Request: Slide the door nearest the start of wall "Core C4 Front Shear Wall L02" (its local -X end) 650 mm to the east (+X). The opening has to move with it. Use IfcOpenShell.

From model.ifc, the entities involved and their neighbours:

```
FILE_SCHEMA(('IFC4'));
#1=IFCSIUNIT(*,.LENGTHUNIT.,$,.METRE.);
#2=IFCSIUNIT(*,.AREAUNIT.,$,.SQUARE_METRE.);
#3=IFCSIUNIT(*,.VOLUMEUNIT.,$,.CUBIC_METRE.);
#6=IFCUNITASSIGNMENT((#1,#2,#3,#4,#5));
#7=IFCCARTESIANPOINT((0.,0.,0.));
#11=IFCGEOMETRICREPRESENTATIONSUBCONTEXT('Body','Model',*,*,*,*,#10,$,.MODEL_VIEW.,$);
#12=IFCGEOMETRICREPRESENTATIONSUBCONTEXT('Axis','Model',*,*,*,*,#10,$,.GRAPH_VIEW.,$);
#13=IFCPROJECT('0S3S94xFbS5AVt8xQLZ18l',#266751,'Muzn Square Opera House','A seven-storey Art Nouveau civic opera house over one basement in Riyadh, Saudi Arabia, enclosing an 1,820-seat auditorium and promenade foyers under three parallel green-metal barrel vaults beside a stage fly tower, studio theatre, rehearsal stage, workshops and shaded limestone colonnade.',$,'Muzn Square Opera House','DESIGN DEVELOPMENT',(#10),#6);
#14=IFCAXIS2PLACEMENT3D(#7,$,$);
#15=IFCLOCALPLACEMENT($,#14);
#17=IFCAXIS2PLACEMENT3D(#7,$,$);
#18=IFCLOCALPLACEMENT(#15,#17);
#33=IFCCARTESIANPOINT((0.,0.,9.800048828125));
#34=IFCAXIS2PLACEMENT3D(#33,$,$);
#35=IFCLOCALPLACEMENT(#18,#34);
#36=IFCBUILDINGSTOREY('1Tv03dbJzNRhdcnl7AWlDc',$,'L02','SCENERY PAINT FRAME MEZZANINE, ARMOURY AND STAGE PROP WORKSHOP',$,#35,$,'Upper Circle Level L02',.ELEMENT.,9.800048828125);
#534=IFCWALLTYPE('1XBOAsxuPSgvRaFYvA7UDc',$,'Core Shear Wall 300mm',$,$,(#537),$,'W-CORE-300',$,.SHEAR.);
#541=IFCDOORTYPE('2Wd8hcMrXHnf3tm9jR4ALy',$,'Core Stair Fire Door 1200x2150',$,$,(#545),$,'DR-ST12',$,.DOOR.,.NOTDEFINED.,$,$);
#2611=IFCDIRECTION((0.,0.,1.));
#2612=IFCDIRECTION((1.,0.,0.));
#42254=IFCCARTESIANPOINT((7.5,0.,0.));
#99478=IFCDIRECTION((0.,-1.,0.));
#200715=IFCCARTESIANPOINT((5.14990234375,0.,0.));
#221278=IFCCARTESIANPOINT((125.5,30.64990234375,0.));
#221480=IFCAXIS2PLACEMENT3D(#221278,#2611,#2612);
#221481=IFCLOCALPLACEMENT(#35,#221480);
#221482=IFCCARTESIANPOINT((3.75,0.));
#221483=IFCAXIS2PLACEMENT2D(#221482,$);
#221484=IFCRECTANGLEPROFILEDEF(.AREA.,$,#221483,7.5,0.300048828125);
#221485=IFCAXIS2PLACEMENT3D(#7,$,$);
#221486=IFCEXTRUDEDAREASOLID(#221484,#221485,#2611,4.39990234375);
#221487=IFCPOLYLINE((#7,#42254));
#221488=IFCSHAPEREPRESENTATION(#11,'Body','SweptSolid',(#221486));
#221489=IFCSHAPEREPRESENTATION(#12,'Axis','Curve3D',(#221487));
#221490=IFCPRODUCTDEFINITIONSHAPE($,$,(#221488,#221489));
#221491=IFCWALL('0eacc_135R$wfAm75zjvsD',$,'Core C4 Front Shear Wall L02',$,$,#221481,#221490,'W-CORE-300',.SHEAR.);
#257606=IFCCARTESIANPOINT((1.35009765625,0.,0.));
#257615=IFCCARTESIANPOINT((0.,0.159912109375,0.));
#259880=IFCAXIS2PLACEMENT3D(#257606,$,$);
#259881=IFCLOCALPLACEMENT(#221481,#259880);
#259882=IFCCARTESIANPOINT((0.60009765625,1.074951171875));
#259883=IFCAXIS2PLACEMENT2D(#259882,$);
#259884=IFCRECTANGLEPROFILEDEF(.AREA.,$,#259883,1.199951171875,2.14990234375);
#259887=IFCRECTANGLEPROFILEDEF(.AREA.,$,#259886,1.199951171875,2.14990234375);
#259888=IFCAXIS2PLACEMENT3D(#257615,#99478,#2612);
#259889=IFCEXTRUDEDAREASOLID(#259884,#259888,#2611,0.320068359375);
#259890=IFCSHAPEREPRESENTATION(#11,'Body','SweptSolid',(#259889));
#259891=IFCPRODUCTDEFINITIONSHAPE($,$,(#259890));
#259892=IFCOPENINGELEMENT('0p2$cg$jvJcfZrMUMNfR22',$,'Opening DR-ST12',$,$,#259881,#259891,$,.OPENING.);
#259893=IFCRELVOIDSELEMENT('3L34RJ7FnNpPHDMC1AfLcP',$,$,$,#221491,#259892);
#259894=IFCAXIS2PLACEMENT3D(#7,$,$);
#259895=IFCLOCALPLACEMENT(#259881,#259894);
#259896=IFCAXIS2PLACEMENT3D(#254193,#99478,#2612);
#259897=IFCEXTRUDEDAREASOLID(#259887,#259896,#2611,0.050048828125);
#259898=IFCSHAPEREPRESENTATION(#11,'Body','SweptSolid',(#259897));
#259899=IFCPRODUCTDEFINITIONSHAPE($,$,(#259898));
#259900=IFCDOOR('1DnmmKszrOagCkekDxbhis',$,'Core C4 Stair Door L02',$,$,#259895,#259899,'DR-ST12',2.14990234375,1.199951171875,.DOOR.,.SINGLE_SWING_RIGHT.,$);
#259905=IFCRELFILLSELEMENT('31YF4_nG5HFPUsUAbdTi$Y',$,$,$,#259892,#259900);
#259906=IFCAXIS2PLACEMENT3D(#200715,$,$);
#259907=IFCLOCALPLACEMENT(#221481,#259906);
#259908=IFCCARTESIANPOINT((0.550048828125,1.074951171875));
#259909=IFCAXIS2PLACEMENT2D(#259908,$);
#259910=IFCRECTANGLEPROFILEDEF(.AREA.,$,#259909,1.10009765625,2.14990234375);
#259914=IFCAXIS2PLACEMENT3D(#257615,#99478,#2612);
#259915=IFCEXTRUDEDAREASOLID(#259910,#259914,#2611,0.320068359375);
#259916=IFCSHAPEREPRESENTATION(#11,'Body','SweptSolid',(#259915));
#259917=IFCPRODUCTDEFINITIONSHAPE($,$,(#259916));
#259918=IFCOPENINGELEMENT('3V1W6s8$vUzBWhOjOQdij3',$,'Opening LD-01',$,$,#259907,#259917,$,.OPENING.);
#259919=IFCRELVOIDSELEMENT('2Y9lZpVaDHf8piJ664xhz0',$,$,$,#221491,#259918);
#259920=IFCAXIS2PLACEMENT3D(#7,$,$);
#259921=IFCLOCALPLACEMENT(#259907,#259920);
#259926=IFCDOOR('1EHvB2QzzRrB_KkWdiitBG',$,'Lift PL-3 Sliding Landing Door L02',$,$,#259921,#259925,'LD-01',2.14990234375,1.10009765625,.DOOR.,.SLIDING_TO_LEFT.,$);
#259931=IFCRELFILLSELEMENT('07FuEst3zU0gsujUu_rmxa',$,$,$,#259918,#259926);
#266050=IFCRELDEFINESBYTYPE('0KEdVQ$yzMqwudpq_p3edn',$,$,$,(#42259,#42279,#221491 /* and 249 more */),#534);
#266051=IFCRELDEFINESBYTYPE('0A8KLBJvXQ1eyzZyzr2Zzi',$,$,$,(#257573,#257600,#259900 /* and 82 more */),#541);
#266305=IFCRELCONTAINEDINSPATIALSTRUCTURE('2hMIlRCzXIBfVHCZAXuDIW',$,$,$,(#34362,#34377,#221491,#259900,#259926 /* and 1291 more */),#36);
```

```python
import ifcopenshell
import ifcopenshell.api.geometry
import ifcopenshell.util.placement

model = ifcopenshell.open("model.ifc")

door = model.by_guid("1DnmmKszrOagCkekDxbhis")
opening = door.FillsVoids[0].RelatingOpeningElement
wall = opening.VoidsElements[0].RelatingBuildingElement

wall_matrix = ifcopenshell.util.placement.get_local_placement(wall.ObjectPlacement)
shift = wall_matrix[:3, 0] * 0.65
before = ifcopenshell.util.placement.get_local_placement(door.ObjectPlacement)[:3, 3].copy()

# The door is placed relative to its opening, so it follows when the opening moves.
matrix = ifcopenshell.util.placement.get_local_placement(opening.ObjectPlacement)
matrix[:3, 3] += shift
ifcopenshell.api.geometry.edit_object_placement(
    model, product=opening, matrix=matrix, is_si=False, should_transform_children=True
)

after = ifcopenshell.util.placement.get_local_placement(door.ObjectPlacement)[:3, 3]
print("door moved by", (after - before).round(3) + 0.0)

model.write("model_edited.ifc")
```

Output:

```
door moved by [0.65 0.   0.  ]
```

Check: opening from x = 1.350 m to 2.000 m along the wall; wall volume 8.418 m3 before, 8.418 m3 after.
